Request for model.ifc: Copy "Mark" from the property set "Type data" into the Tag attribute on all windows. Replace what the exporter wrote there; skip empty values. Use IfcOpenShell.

First a look at what the model holds.

```python
import ifcopenshell
import ifcopenshell.util.element

model = ifcopenshell.open("model.ifc")
print(model.schema)
windows = model.by_type("IfcWindow")
print(len(windows), "windows")
for e in windows[:8]:
    source = ifcopenshell.util.element.get_pset(e, "Type data", "Mark")
    target = e.Tag
    print(e.id(), repr(source), repr(target), sep=" | ")
```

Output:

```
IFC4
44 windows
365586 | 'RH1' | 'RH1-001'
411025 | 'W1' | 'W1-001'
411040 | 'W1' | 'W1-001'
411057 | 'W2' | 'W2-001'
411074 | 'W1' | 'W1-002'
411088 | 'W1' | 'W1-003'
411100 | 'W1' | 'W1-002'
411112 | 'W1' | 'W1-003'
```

```python
import ifcopenshell
import ifcopenshell.util.element

model = ifcopenshell.open("model.ifc")

count = 0
for e in model.by_type("IfcWindow"):
    value = ifcopenshell.util.element.get_pset(e, "Type data", "Mark")
    current = e.Tag
    if not value or not value.strip() or current == value:
        continue
    e.Tag = value
    count += 1

print(count, "windows updated")

model.write("model_v2.ifc")
```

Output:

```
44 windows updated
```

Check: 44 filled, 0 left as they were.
